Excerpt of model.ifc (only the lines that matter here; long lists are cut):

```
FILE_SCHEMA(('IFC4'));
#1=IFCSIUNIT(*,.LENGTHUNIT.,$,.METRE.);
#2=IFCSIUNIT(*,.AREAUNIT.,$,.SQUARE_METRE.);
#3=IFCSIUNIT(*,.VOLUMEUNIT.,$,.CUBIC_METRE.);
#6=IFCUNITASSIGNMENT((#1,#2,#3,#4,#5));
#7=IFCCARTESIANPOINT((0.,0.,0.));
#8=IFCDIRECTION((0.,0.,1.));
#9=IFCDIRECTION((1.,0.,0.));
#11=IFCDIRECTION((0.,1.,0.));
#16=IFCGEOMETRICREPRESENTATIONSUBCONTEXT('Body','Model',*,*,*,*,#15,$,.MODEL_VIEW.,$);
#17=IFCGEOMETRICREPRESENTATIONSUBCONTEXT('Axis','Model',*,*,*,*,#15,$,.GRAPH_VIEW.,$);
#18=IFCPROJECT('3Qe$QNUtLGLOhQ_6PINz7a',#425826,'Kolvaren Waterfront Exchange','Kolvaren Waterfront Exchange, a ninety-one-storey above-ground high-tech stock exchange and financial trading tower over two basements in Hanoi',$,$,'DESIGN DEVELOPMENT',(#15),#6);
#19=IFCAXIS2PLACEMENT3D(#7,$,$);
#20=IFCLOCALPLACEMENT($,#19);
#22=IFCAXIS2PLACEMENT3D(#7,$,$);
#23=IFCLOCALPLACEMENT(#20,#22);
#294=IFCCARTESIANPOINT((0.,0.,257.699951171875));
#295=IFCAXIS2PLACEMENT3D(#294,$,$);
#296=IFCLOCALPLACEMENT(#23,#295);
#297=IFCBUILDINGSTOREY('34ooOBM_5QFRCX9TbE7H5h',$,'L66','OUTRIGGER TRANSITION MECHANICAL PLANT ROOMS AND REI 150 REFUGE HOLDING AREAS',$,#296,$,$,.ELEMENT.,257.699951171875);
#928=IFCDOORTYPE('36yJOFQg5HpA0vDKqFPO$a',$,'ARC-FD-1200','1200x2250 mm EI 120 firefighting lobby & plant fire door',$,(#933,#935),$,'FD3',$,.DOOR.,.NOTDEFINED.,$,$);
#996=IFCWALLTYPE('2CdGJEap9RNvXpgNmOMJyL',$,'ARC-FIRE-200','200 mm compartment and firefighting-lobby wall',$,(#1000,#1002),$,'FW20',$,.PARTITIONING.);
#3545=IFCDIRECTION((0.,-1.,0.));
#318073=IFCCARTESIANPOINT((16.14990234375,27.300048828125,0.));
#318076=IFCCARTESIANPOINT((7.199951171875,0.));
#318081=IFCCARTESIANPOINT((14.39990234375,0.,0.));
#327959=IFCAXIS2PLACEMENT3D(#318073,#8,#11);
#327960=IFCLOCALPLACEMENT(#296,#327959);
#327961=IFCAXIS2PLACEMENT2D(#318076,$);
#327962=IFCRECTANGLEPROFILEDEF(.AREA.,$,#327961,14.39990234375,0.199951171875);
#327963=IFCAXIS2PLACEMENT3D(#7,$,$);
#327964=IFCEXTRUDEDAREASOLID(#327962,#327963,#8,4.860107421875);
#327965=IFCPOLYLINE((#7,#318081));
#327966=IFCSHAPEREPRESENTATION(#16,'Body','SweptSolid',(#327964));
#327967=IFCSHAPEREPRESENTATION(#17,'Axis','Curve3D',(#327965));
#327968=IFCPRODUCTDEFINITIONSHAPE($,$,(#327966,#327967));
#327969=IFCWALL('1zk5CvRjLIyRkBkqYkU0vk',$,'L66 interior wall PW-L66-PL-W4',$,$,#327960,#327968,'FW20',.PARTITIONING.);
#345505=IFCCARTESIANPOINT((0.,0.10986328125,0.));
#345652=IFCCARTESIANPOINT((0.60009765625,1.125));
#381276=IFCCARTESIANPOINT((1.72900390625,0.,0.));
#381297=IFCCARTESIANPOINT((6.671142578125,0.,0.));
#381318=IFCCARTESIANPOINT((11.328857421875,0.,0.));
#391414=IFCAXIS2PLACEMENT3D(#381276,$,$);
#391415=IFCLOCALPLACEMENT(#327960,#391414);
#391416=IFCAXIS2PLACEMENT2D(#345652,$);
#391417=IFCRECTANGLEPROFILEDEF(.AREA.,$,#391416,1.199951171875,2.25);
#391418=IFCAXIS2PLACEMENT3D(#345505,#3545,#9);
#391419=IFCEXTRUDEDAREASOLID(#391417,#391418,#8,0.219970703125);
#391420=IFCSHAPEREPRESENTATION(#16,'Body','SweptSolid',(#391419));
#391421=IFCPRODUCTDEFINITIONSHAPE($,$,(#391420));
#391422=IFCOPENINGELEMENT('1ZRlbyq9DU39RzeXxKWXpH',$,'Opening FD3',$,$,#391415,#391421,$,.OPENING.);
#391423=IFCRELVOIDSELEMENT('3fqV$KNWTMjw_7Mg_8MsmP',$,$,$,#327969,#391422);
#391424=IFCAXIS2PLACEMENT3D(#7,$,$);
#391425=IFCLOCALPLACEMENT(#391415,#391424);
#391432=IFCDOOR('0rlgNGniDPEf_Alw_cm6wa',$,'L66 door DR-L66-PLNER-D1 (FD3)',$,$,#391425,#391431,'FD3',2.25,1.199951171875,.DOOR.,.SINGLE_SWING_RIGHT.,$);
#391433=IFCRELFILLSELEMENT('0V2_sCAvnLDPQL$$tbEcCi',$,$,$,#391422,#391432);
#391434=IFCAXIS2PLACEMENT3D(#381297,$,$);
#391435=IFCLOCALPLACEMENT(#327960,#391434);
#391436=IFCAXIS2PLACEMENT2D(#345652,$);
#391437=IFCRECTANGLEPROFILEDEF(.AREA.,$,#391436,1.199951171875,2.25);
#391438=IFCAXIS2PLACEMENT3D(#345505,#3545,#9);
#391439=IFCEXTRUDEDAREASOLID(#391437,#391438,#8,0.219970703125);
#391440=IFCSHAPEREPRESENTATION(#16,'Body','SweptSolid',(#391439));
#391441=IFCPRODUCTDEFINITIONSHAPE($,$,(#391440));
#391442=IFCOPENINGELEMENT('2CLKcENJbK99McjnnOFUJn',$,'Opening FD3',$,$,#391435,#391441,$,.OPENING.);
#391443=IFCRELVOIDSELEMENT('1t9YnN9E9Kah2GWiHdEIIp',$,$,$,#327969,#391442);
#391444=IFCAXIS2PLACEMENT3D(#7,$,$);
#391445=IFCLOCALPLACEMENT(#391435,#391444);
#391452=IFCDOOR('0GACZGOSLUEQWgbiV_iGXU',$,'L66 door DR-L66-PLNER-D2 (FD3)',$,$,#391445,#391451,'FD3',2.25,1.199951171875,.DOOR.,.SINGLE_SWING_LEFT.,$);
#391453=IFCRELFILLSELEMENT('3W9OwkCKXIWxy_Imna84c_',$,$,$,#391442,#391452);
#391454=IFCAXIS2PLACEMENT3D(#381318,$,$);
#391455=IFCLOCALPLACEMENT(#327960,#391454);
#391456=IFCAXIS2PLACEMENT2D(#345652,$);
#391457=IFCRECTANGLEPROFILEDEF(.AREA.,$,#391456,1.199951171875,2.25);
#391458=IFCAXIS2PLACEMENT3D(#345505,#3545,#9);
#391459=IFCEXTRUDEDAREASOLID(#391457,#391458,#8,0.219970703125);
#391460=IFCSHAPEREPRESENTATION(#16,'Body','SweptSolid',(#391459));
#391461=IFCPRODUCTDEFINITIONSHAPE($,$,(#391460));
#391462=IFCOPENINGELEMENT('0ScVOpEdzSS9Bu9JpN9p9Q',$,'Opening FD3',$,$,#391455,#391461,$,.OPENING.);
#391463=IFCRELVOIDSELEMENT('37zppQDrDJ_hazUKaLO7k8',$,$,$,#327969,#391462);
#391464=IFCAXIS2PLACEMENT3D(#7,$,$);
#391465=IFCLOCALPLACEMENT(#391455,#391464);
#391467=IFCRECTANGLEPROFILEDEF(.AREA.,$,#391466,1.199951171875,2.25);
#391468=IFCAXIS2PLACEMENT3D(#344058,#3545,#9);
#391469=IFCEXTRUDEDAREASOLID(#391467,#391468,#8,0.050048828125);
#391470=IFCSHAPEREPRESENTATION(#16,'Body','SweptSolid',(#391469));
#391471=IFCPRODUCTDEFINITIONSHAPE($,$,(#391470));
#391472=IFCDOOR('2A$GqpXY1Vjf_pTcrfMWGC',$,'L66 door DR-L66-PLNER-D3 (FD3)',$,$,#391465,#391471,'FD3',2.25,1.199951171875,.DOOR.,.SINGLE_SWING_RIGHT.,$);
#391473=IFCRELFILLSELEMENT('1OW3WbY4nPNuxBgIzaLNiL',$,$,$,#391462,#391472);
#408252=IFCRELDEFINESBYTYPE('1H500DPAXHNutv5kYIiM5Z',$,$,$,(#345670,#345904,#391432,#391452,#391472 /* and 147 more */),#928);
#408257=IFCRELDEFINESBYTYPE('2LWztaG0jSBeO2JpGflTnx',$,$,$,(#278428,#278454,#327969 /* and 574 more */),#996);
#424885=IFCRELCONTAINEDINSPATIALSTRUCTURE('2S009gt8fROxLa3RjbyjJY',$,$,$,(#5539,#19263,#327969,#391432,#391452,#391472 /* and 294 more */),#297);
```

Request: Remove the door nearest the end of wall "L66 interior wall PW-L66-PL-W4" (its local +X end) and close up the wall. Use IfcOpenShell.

```python
import ifcopenshell
import ifcopenshell.api.feature
import ifcopenshell.api.root
import ifcopenshell.geom
import ifcopenshell.util.shape

model = ifcopenshell.open("model.ifc")
settings = ifcopenshell.geom.settings()


def volume(element):
    """Net volume in cubic metres, openings subtracted."""
    shape = ifcopenshell.geom.create_shape(settings, element)
    return ifcopenshell.util.shape.get_volume(shape.geometry)


door = model.by_id(391472)
opening = door.FillsVoids[0].RelatingOpeningElement
wall = opening.VoidsElements[0].RelatingBuildingElement
before = volume(wall)

ifcopenshell.api.root.remove_product(model, product=door)
ifcopenshell.api.feature.remove_feature(model, feature=opening)

after = volume(wall)

print(f"wall volume {before:.3f} -> {after:.3f} m3")

model.write("model_v2.ifc")
```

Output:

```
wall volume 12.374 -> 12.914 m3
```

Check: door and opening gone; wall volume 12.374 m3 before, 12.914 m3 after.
